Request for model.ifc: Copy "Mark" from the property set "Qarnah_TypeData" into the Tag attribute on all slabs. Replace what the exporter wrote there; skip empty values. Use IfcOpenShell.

First a look at what the model holds.

```python
import ifcopenshell
import ifcopenshell.util.element

model = ifcopenshell.open("model.ifc")
print(model.schema)
slabs = model.by_type("IfcSlab")
print(len(slabs), "slabs")
for e in slabs[:8]:
    source = ifcopenshell.util.element.get_pset(e, "Qarnah_TypeData", "Mark")
    target = e.Tag
    print(e.id(), repr(source), repr(target), sep=" | ")
```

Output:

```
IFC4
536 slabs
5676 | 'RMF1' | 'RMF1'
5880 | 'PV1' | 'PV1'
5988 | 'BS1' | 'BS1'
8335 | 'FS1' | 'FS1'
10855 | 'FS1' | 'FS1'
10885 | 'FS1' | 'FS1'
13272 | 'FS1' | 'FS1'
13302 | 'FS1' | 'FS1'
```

```python
import ifcopenshell
import ifcopenshell.util.element

model = ifcopenshell.open("model.ifc")

count = 0
for e in model.by_type("IfcSlab"):
    value = ifcopenshell.util.element.get_pset(e, "Qarnah_TypeData", "Mark")
    current = e.Tag
    if not value or not value.strip() or current == value:
        continue
    e.Tag = value
    count += 1

print(count, "slabs updated")

model.write("model_rev.ifc")
```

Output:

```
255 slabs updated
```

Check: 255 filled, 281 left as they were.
